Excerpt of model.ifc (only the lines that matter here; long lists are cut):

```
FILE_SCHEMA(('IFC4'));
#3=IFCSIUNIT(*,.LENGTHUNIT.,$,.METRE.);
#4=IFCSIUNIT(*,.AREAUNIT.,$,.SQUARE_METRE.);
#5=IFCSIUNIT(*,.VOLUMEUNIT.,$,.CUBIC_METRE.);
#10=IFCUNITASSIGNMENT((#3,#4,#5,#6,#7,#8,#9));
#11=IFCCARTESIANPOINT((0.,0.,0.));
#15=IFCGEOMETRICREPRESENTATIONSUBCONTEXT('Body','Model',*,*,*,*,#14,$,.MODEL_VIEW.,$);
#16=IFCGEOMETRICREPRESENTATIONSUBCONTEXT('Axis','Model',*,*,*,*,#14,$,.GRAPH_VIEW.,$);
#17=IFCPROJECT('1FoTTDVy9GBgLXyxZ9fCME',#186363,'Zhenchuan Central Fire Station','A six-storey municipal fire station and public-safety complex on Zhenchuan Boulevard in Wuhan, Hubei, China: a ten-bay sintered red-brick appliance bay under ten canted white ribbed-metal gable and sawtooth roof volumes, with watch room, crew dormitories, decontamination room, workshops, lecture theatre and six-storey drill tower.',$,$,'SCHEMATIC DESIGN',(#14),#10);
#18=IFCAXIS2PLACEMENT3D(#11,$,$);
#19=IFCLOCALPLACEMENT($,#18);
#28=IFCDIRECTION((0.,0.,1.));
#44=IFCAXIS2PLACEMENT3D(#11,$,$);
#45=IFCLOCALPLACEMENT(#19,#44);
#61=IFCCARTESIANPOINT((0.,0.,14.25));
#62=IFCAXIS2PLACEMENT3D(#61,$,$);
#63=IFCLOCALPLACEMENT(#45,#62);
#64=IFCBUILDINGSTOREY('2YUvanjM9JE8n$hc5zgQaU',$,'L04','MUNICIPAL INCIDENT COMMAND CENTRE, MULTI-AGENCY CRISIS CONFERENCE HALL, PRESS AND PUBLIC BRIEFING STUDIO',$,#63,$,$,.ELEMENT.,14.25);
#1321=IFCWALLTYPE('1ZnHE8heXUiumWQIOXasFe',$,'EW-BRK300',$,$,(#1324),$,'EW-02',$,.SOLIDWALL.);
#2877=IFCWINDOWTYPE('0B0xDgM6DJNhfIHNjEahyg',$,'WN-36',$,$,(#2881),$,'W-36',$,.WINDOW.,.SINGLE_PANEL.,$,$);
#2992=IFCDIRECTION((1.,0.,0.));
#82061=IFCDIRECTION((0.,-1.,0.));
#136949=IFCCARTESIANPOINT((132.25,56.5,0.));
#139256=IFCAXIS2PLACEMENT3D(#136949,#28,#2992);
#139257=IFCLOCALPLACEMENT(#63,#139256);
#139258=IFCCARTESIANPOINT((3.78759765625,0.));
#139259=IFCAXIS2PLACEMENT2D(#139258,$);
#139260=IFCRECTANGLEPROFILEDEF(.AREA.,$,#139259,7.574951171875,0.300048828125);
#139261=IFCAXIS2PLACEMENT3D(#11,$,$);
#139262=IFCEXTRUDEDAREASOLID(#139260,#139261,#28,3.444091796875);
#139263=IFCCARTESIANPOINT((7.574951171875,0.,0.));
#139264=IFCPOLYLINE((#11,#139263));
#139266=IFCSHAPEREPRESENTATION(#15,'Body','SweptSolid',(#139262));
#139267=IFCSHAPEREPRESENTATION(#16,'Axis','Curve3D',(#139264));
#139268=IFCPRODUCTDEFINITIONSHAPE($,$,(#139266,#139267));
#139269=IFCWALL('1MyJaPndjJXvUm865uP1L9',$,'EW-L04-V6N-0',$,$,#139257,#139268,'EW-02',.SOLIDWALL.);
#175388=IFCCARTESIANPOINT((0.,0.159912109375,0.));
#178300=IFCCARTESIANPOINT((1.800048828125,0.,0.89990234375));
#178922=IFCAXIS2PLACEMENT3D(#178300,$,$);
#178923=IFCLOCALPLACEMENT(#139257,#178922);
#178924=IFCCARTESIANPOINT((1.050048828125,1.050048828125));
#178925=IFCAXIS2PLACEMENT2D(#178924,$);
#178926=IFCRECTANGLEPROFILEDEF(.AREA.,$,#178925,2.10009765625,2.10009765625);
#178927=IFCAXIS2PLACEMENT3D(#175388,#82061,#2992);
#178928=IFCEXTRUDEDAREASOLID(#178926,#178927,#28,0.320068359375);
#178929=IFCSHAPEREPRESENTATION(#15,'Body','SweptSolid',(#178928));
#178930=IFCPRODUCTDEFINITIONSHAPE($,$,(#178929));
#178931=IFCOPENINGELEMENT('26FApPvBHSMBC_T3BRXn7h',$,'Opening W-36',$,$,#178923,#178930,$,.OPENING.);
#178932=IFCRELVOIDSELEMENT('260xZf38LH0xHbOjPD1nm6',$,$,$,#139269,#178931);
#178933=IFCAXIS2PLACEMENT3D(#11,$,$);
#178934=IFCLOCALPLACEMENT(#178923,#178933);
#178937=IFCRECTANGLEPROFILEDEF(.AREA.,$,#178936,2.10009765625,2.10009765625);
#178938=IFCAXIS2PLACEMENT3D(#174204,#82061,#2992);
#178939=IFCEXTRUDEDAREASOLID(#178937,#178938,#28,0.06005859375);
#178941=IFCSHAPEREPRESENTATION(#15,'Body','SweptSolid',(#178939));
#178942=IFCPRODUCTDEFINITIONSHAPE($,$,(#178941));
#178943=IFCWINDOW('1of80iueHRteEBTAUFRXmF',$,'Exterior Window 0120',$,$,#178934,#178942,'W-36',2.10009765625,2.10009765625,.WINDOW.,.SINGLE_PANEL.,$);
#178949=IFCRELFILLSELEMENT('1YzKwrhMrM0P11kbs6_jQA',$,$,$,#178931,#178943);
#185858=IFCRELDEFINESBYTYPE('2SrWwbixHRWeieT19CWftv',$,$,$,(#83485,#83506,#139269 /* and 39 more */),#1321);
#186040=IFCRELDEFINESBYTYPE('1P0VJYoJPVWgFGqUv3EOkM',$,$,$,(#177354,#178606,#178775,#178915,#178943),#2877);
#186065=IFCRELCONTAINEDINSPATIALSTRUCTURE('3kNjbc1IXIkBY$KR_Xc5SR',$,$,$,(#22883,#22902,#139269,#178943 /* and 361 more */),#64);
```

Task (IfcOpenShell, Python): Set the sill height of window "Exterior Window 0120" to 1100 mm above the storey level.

```python
import numpy as np
import ifcopenshell
import ifcopenshell.api.geometry
import ifcopenshell.geom
import ifcopenshell.util.element
import ifcopenshell.util.placement
import ifcopenshell.util.shape
import ifcopenshell.util.unit

model = ifcopenshell.open("model.ifc")
unit_scale = ifcopenshell.util.unit.calculate_unit_scale(model)

window = model.by_id(178943)
opening = window.FillsVoids[0].RelatingOpeningElement
storey = ifcopenshell.util.element.get_container(window, ifc_class="IfcBuildingStorey")
level = ifcopenshell.util.placement.get_local_placement(storey.ObjectPlacement)[2, 3]

# The opening's origin need not be at the sill, so measure its lowest point.
shape = ifcopenshell.geom.create_shape(ifcopenshell.geom.settings(), opening)
bottom = ifcopenshell.util.shape.get_shape_bottom_elevation(shape, shape.geometry) / unit_scale
dz = level + 1.1 / unit_scale - bottom

shift = np.array([0.0, 0.0, dz])
# The window is placed relative to its opening, so it follows when the opening moves.
matrix = ifcopenshell.util.placement.get_local_placement(opening.ObjectPlacement)
matrix[:3, 3] += shift
ifcopenshell.api.geometry.edit_object_placement(
    model, product=opening, matrix=matrix, is_si=False, should_transform_children=True
)

print(f"moved by {dz * unit_scale:+.3f} m")

model.write("model_rev.ifc")
```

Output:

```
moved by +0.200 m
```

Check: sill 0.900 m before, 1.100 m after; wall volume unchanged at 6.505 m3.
